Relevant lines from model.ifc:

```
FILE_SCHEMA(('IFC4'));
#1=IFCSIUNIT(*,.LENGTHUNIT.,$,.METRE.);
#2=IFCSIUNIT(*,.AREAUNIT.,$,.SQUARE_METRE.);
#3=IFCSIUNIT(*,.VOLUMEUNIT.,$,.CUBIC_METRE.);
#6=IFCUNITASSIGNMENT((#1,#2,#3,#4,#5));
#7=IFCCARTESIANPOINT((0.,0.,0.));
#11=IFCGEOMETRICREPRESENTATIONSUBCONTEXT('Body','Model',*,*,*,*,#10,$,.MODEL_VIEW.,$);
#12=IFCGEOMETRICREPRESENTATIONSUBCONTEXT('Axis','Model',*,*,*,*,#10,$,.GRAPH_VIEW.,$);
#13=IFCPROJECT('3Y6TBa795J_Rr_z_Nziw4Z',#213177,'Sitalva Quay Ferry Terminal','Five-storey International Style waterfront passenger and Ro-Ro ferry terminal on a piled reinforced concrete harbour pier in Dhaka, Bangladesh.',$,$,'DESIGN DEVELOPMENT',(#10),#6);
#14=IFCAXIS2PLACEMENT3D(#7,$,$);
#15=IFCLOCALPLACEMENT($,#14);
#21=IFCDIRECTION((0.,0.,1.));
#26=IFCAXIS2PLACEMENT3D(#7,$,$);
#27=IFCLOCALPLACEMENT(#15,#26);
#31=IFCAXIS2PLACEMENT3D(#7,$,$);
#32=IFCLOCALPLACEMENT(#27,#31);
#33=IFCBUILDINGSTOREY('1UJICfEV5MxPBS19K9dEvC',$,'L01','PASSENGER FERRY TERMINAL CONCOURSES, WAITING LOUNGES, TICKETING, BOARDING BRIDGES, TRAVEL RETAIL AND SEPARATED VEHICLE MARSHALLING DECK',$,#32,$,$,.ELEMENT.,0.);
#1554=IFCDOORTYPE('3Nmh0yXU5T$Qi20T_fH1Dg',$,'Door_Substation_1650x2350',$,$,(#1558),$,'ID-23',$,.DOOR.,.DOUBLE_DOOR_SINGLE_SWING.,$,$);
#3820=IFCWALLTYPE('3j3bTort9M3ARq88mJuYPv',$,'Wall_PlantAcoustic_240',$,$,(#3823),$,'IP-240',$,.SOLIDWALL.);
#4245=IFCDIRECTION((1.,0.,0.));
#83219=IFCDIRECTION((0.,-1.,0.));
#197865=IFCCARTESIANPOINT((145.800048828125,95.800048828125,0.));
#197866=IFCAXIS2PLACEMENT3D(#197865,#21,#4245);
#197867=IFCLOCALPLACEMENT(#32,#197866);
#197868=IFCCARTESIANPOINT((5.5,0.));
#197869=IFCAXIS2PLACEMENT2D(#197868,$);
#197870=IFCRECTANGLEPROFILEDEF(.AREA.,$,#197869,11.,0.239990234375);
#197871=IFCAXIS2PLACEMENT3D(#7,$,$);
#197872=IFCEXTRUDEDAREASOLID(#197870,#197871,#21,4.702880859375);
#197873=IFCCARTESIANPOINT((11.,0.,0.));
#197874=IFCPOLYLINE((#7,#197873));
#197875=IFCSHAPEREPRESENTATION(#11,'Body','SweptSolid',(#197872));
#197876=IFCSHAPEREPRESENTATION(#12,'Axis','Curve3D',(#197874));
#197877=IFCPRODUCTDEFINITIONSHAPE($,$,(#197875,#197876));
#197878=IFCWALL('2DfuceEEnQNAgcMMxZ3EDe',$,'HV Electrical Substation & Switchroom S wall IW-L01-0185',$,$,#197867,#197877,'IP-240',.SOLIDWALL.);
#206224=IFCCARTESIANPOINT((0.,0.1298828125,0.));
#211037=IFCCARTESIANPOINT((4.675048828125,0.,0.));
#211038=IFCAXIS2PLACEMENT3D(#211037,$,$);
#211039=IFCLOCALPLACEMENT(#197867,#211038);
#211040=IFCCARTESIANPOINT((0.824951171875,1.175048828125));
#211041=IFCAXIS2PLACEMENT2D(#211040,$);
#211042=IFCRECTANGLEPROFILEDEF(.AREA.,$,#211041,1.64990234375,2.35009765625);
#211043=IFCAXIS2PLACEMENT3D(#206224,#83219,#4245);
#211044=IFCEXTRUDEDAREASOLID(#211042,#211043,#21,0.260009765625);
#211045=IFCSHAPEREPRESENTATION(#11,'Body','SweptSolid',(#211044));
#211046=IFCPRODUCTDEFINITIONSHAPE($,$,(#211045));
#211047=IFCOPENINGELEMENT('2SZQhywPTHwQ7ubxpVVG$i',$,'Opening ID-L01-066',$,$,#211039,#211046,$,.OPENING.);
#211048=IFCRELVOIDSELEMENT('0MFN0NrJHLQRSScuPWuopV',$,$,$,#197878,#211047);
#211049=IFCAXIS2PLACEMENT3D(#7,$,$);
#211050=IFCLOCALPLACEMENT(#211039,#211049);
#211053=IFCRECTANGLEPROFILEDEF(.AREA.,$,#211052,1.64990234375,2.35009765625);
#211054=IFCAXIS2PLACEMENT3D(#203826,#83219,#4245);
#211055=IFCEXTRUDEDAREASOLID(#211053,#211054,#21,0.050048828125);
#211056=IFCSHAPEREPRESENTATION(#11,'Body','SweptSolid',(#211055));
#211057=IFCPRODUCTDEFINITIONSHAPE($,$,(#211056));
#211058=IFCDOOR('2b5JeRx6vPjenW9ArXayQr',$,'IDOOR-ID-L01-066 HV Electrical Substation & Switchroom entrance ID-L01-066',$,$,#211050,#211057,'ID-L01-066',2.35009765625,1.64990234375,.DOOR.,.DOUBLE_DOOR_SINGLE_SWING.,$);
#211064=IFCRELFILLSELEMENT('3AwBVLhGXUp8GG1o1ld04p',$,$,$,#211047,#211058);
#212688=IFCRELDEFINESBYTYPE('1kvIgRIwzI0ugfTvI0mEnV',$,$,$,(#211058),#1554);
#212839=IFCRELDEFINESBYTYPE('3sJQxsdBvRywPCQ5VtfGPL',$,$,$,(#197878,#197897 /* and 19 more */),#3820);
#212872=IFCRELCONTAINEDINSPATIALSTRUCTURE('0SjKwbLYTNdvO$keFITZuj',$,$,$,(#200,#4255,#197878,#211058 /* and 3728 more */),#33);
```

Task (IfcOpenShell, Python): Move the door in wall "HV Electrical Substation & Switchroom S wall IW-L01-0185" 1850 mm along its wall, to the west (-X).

```python
import ifcopenshell
import ifcopenshell.api.geometry
import ifcopenshell.util.placement

model = ifcopenshell.open("model.ifc")

door = model.by_guid("2b5JeRx6vPjenW9ArXayQr")
opening = door.FillsVoids[0].RelatingOpeningElement
wall = opening.VoidsElements[0].RelatingBuildingElement

wall_matrix = ifcopenshell.util.placement.get_local_placement(wall.ObjectPlacement)
shift = wall_matrix[:3, 0] * -1.85
before = ifcopenshell.util.placement.get_local_placement(door.ObjectPlacement)[:3, 3].copy()

# The door is placed relative to its opening, so it follows when the opening moves.
matrix = ifcopenshell.util.placement.get_local_placement(opening.ObjectPlacement)
matrix[:3, 3] += shift
ifcopenshell.api.geometry.edit_object_placement(
    model, product=opening, matrix=matrix, is_si=False, should_transform_children=True
)

after = ifcopenshell.util.placement.get_local_placement(door.ObjectPlacement)[:3, 3]
print("door moved by", (after - before).round(3) + 0.0)

model.write("model_edited.ifc")
```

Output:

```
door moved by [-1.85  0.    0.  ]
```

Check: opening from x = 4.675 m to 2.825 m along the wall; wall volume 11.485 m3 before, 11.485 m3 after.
